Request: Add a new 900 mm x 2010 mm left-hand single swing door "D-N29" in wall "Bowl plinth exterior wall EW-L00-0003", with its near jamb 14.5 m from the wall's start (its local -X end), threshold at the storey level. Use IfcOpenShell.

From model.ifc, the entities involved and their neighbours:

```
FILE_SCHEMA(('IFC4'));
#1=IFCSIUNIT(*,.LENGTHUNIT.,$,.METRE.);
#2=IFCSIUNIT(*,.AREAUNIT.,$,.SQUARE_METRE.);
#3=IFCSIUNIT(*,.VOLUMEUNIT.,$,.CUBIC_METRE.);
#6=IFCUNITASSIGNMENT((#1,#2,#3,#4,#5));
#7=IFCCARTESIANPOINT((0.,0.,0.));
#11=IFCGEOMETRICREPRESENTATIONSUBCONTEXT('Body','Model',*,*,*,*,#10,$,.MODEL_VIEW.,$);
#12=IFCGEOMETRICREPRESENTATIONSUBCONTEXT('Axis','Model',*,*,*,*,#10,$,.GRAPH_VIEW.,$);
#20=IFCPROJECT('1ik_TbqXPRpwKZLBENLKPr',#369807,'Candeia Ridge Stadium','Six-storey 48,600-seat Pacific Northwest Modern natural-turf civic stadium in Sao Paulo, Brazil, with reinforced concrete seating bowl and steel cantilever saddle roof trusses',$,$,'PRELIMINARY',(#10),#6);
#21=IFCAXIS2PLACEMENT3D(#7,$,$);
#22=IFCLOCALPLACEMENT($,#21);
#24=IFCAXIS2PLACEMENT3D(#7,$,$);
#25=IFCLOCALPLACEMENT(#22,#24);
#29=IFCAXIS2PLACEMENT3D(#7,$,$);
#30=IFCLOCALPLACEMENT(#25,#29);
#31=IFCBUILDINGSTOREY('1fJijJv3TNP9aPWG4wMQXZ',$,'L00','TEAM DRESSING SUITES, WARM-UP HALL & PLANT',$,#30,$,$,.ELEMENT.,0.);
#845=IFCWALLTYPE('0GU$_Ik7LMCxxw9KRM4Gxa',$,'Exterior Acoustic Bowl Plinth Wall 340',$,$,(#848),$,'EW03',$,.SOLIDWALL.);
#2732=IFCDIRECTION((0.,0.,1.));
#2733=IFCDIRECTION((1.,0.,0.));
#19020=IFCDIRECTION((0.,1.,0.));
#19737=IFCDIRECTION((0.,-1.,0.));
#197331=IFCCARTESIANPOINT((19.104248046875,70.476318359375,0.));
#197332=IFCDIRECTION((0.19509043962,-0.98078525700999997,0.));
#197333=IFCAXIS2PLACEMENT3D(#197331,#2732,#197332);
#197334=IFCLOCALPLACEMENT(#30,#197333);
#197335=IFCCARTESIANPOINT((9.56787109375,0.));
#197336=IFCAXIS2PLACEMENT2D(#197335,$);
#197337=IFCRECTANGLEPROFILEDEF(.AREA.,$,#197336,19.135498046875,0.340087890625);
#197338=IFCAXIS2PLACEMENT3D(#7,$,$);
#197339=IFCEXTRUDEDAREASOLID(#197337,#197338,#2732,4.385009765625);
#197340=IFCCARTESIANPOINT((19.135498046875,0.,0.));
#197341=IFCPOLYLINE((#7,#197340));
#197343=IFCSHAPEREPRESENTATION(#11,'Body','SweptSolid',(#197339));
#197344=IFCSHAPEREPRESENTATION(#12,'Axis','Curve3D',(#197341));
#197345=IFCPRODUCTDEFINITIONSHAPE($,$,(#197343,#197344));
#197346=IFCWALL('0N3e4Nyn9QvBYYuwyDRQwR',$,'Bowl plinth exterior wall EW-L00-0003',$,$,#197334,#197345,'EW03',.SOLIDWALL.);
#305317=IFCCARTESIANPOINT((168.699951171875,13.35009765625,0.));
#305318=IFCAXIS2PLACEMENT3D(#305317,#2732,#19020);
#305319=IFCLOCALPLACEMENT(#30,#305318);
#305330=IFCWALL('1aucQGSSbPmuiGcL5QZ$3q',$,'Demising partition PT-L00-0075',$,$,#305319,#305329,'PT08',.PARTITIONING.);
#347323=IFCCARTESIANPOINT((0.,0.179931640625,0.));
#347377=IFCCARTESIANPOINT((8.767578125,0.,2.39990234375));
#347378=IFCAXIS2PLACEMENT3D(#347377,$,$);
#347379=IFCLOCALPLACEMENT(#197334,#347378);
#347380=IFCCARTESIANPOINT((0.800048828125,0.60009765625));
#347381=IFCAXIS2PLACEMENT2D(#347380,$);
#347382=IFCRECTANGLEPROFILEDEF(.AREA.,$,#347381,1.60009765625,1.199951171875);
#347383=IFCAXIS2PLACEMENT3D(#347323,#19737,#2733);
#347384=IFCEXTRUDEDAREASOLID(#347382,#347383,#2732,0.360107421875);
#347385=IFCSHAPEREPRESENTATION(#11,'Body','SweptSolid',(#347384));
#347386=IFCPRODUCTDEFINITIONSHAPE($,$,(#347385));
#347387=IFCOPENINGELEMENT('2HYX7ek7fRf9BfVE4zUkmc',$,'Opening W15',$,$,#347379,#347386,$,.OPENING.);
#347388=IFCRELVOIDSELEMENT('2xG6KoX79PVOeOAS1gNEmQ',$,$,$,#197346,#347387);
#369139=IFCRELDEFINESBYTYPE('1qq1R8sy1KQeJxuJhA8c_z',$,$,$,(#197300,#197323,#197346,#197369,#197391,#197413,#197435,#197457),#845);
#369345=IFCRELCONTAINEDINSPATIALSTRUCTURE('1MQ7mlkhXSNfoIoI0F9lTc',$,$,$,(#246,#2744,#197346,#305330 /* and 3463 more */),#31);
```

```python
import numpy as np
import ifcopenshell
import ifcopenshell.api.feature
import ifcopenshell.api.geometry
import ifcopenshell.api.root
import ifcopenshell.api.spatial
import ifcopenshell.geom
import ifcopenshell.util.element
import ifcopenshell.util.placement
import ifcopenshell.util.representation
import ifcopenshell.util.shape
import ifcopenshell.util.unit

model = ifcopenshell.open("model.ifc")
unit_scale = ifcopenshell.util.unit.calculate_unit_scale(model)
settings = ifcopenshell.geom.settings()


def volume(element):
    """Net volume in cubic metres, openings subtracted."""
    shape = ifcopenshell.geom.create_shape(settings, element)
    return ifcopenshell.util.shape.get_volume(shape.geometry)


wall = model.by_guid("0N3e4Nyn9QvBYYuwyDRQwR")
storey = ifcopenshell.util.element.get_container(wall, ifc_class="IfcBuildingStorey")
context = ifcopenshell.util.representation.get_context(model, "Model", "Body", "MODEL_VIEW")
before = volume(wall)

width, height, from_end, sill = 0.9, 2.01, 14.5, 0.0  # metres

# The wall runs along its own X axis, and the end named is its -X end.
wall_shape = ifcopenshell.geom.create_shape(settings, wall)
x, y, z = ifcopenshell.util.shape.get_vertices(wall_shape.geometry).T
start = x.min() + from_end
face, thickness = float(y.min()), float(y.max() - y.min())
wall_matrix = ifcopenshell.util.placement.get_local_placement(wall.ObjectPlacement)
level = ifcopenshell.util.placement.get_local_placement(storey.ObjectPlacement)[2, 3]


def in_wall(x, y):
    """Placement at x, y metres in the wall's axes, at sill height."""
    matrix = wall_matrix.copy()
    matrix[:, 3] = wall_matrix @ np.array([x / unit_scale, y / unit_scale, 0.0, 1.0])
    matrix[2, 3] = level + sill / unit_scale
    return matrix


# Opening: a box that overshoots both wall faces by 50 mm.
opening = ifcopenshell.api.root.create_entity(model, ifc_class="IfcOpeningElement", predefined_type="OPENING")
box = ifcopenshell.api.geometry.add_wall_representation(
    model, context=context, length=width, height=height, thickness=thickness + 0.1
)
ifcopenshell.api.geometry.assign_representation(model, product=opening, representation=box)
ifcopenshell.api.geometry.edit_object_placement(model, product=opening, matrix=in_wall(start, face - 0.05), is_si=False)
ifcopenshell.api.feature.add_feature(model, feature=opening, element=wall)

door = ifcopenshell.api.root.create_entity(model, ifc_class="IfcDoor", name="D-N29", predefined_type="DOOR")
door.OverallWidth, door.OverallHeight = width / unit_scale, height / unit_scale
door.OperationType = "SINGLE_SWING_LEFT"
body = ifcopenshell.api.geometry.add_door_representation(
    model,
    context=context,
    overall_width=door.OverallWidth,
    overall_height=door.OverallHeight,
    operation_type="SINGLE_SWING_LEFT",
    lining_properties={"LiningDepth": thickness / unit_scale, "ThresholdDepth": thickness / unit_scale},
)
ifcopenshell.api.geometry.assign_representation(model, product=door, representation=body)
ifcopenshell.api.spatial.assign_container(model, products=[door], relating_structure=storey)
ifcopenshell.api.feature.add_filling(model, opening=opening, element=door)

# The lining spans the wall, so the door starts at the wall face.
ifcopenshell.api.geometry.edit_object_placement(model, product=door, matrix=in_wall(start, face), is_si=False)

after = volume(wall)

print(f"wall volume {before:.3f} -> {after:.3f} m3")

model.write("model_updated.ifc")
```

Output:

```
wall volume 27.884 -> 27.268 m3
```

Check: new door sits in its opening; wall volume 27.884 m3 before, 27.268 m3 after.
